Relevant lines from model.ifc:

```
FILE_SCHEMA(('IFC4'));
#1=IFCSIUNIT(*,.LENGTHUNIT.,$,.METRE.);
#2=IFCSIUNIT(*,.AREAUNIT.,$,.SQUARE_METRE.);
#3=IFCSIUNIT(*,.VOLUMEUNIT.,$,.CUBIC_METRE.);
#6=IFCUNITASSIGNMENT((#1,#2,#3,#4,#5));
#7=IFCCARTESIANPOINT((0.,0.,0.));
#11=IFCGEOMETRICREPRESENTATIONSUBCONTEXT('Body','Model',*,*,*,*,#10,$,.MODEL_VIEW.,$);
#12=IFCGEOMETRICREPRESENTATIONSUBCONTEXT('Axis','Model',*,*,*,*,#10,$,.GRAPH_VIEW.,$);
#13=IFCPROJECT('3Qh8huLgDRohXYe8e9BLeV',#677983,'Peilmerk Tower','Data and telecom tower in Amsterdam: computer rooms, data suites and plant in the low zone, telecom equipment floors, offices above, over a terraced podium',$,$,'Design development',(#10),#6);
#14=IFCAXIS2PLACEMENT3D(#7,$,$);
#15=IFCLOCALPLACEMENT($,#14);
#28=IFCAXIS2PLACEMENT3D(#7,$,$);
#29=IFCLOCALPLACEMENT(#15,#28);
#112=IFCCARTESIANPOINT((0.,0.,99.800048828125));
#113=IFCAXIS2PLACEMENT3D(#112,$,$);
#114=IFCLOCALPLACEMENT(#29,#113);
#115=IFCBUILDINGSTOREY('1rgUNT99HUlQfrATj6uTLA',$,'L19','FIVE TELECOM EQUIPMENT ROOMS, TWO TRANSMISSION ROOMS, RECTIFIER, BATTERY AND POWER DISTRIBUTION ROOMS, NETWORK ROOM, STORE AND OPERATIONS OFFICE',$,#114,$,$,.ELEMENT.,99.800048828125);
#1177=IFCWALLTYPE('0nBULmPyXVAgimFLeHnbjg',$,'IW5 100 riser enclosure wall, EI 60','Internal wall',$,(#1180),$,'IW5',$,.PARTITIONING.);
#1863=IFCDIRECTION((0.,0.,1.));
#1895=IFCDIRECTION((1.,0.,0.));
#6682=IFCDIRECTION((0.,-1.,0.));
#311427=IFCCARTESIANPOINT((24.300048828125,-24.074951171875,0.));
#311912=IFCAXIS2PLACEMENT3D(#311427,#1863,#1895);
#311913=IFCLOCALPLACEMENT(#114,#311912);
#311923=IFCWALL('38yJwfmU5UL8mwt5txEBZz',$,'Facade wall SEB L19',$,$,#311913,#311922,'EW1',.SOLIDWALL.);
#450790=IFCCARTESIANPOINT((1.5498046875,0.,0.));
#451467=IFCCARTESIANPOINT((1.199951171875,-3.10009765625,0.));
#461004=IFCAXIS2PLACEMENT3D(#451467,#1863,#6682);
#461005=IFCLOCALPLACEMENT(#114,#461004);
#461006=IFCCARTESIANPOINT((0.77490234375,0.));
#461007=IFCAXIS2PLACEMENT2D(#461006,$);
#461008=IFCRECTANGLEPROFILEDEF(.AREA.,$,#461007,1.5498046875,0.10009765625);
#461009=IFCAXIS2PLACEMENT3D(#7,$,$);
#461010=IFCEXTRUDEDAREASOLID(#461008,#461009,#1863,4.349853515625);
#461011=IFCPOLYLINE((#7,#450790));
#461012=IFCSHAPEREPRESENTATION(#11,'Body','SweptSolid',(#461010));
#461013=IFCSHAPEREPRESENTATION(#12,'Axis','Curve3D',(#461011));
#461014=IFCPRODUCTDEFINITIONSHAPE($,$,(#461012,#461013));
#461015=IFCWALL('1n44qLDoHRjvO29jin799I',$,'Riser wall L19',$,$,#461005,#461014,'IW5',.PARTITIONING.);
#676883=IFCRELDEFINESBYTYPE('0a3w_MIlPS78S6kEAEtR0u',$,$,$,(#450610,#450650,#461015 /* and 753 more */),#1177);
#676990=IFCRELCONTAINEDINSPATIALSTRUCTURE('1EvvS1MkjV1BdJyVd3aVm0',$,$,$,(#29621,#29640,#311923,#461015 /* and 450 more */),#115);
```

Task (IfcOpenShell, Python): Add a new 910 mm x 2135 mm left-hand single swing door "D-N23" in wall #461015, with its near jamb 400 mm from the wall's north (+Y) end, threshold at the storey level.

```python
import numpy as np
import ifcopenshell
import ifcopenshell.api.feature
import ifcopenshell.api.geometry
import ifcopenshell.api.root
import ifcopenshell.api.spatial
import ifcopenshell.geom
import ifcopenshell.util.element
import ifcopenshell.util.placement
import ifcopenshell.util.representation
import ifcopenshell.util.shape
import ifcopenshell.util.unit

model = ifcopenshell.open("model.ifc")
unit_scale = ifcopenshell.util.unit.calculate_unit_scale(model)
settings = ifcopenshell.geom.settings()


def volume(element):
    """Net volume in cubic metres, openings subtracted."""
    shape = ifcopenshell.geom.create_shape(settings, element)
    return ifcopenshell.util.shape.get_volume(shape.geometry)


wall = model.by_guid("1n44qLDoHRjvO29jin799I")
storey = ifcopenshell.util.element.get_container(wall, ifc_class="IfcBuildingStorey")
context = ifcopenshell.util.representation.get_context(model, "Model", "Body", "MODEL_VIEW")
before = volume(wall)

width, height, from_end, sill = 0.91, 2.135, 0.4, 0.0  # metres

# The wall runs along its own X axis, and the end named is its -X end.
wall_shape = ifcopenshell.geom.create_shape(settings, wall)
x, y, z = ifcopenshell.util.shape.get_vertices(wall_shape.geometry).T
start = x.min() + from_end
face, thickness = float(y.min()), float(y.max() - y.min())
wall_matrix = ifcopenshell.util.placement.get_local_placement(wall.ObjectPlacement)
level = ifcopenshell.util.placement.get_local_placement(storey.ObjectPlacement)[2, 3]


def in_wall(x, y):
    """Placement at x, y metres in the wall's axes, at sill height."""
    matrix = wall_matrix.copy()
    matrix[:, 3] = wall_matrix @ np.array([x / unit_scale, y / unit_scale, 0.0, 1.0])
    matrix[2, 3] = level + sill / unit_scale
    return matrix


# Opening: a box that overshoots both wall faces by 50 mm.
opening = ifcopenshell.api.root.create_entity(model, ifc_class="IfcOpeningElement", predefined_type="OPENING")
box = ifcopenshell.api.geometry.add_wall_representation(
    model, context=context, length=width, height=height, thickness=thickness + 0.1
)
ifcopenshell.api.geometry.assign_representation(model, product=opening, representation=box)
ifcopenshell.api.geometry.edit_object_placement(model, product=opening, matrix=in_wall(start, face - 0.05), is_si=False)
ifcopenshell.api.feature.add_feature(model, feature=opening, element=wall)

door = ifcopenshell.api.root.create_entity(model, ifc_class="IfcDoor", name="D-N23", predefined_type="DOOR")
door.OverallWidth, door.OverallHeight = width / unit_scale, height / unit_scale
door.OperationType = "SINGLE_SWING_LEFT"
body = ifcopenshell.api.geometry.add_door_representation(
    model,
    context=context,
    overall_width=door.OverallWidth,
    overall_height=door.OverallHeight,
    operation_type="SINGLE_SWING_LEFT",
    lining_properties={"LiningDepth": thickness / unit_scale, "ThresholdDepth": thickness / unit_scale},
)
ifcopenshell.api.geometry.assign_representation(model, product=door, representation=body)
ifcopenshell.api.spatial.assign_container(model, products=[door], relating_structure=storey)
ifcopenshell.api.feature.add_filling(model, opening=opening, element=door)

# The lining spans the wall, so the door starts at the wall face.
ifcopenshell.api.geometry.edit_object_placement(model, product=door, matrix=in_wall(start, face), is_si=False)

after = volume(wall)

print(f"wall volume {before:.3f} -> {after:.3f} m3")

model.write("model-out.ifc")
```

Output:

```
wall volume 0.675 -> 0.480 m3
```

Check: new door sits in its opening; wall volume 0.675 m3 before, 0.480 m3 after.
